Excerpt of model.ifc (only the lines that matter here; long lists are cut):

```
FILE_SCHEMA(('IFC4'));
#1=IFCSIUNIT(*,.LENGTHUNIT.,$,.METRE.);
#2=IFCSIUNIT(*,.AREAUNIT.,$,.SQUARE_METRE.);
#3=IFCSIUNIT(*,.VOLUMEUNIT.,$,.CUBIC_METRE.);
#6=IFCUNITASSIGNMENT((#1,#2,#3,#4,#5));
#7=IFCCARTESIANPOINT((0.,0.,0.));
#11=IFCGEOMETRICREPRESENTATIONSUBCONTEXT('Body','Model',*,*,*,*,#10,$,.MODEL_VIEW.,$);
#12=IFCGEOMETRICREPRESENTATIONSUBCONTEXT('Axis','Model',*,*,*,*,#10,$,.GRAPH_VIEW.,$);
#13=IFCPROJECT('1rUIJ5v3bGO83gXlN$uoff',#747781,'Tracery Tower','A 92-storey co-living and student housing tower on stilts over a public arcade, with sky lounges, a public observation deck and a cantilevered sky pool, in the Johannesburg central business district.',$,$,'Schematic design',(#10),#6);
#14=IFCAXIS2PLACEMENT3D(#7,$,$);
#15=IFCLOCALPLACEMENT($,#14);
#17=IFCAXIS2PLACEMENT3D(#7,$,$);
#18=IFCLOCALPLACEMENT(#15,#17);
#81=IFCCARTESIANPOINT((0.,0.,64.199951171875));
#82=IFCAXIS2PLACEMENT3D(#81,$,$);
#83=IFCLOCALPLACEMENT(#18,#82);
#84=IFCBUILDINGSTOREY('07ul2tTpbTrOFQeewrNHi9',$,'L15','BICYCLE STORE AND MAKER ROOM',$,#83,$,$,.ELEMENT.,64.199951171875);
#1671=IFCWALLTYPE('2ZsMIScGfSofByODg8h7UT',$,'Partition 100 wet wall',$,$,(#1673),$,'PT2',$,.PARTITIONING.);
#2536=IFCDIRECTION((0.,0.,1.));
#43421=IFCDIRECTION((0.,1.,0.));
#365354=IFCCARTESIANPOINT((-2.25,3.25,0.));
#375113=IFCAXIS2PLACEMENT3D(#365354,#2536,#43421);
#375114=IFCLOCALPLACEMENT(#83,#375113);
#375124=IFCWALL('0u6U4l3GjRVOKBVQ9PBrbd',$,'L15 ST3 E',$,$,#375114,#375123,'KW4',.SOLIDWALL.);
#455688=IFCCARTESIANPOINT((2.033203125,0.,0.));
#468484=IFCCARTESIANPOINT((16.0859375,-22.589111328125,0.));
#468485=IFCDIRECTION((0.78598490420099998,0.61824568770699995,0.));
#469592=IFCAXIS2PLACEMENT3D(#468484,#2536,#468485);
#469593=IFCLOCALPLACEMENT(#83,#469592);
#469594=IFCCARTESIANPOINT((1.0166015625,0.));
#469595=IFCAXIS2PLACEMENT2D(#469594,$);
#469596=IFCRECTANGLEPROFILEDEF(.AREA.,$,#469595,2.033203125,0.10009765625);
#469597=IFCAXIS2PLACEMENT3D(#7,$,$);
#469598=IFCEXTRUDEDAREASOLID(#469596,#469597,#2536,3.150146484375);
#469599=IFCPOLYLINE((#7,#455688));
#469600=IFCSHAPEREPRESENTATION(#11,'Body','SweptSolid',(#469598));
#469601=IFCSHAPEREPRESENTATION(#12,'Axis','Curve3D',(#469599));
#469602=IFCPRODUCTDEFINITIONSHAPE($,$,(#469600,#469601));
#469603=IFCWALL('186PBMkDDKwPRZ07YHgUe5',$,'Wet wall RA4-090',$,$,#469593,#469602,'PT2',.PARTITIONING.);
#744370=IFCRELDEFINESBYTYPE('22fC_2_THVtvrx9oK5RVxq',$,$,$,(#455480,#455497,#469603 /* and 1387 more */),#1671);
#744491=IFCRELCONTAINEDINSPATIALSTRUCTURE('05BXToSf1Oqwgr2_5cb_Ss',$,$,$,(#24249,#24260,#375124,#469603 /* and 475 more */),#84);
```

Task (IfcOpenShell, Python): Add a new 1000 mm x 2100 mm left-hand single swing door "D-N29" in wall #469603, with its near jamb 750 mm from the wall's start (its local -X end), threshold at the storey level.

```python
import numpy as np
import ifcopenshell
import ifcopenshell.api.feature
import ifcopenshell.api.geometry
import ifcopenshell.api.root
import ifcopenshell.api.spatial
import ifcopenshell.geom
import ifcopenshell.util.element
import ifcopenshell.util.placement
import ifcopenshell.util.representation
import ifcopenshell.util.shape
import ifcopenshell.util.unit

model = ifcopenshell.open("model.ifc")
unit_scale = ifcopenshell.util.unit.calculate_unit_scale(model)
settings = ifcopenshell.geom.settings()


def volume(element):
    """Net volume in cubic metres, openings subtracted."""
    shape = ifcopenshell.geom.create_shape(settings, element)
    return ifcopenshell.util.shape.get_volume(shape.geometry)


wall = model.by_id(469603)
storey = ifcopenshell.util.element.get_container(wall, ifc_class="IfcBuildingStorey")
context = ifcopenshell.util.representation.get_context(model, "Model", "Body", "MODEL_VIEW")
before = volume(wall)

width, height, from_end, sill = 1, 2.1, 0.75, 0.0  # metres

# The wall runs along its own X axis, and the end named is its -X end.
wall_shape = ifcopenshell.geom.create_shape(settings, wall)
x, y, z = ifcopenshell.util.shape.get_vertices(wall_shape.geometry).T
start = x.min() + from_end
face, thickness = float(y.min()), float(y.max() - y.min())
wall_matrix = ifcopenshell.util.placement.get_local_placement(wall.ObjectPlacement)
level = ifcopenshell.util.placement.get_local_placement(storey.ObjectPlacement)[2, 3]


def in_wall(x, y):
    """Placement at x, y metres in the wall's axes, at sill height."""
    matrix = wall_matrix.copy()
    matrix[:, 3] = wall_matrix @ np.array([x / unit_scale, y / unit_scale, 0.0, 1.0])
    matrix[2, 3] = level + sill / unit_scale
    return matrix


# Opening: a box that overshoots both wall faces by 50 mm.
opening = ifcopenshell.api.root.create_entity(model, ifc_class="IfcOpeningElement", predefined_type="OPENING")
box = ifcopenshell.api.geometry.add_wall_representation(
    model, context=context, length=width, height=height, thickness=thickness + 0.1
)
ifcopenshell.api.geometry.assign_representation(model, product=opening, representation=box)
ifcopenshell.api.geometry.edit_object_placement(model, product=opening, matrix=in_wall(start, face - 0.05), is_si=False)
ifcopenshell.api.feature.add_feature(model, feature=opening, element=wall)

door = ifcopenshell.api.root.create_entity(model, ifc_class="IfcDoor", name="D-N29", predefined_type="DOOR")
door.OverallWidth, door.OverallHeight = width / unit_scale, height / unit_scale
door.OperationType = "SINGLE_SWING_LEFT"
body = ifcopenshell.api.geometry.add_door_representation(
    model,
    context=context,
    overall_width=door.OverallWidth,
    overall_height=door.OverallHeight,
    operation_type="SINGLE_SWING_LEFT",
    lining_properties={"LiningDepth": thickness / unit_scale, "ThresholdDepth": thickness / unit_scale},
)
ifcopenshell.api.geometry.assign_representation(model, product=door, representation=body)
ifcopenshell.api.spatial.assign_container(model, products=[door], relating_structure=storey)
ifcopenshell.api.feature.add_filling(model, opening=opening, element=door)

# The lining spans the wall, so the door starts at the wall face.
ifcopenshell.api.geometry.edit_object_placement(model, product=door, matrix=in_wall(start, face), is_si=False)

after = volume(wall)

print(f"wall volume {before:.3f} -> {after:.3f} m3")

model.write("model_rev.ifc")
```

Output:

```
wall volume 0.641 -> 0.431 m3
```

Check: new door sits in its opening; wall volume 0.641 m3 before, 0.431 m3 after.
